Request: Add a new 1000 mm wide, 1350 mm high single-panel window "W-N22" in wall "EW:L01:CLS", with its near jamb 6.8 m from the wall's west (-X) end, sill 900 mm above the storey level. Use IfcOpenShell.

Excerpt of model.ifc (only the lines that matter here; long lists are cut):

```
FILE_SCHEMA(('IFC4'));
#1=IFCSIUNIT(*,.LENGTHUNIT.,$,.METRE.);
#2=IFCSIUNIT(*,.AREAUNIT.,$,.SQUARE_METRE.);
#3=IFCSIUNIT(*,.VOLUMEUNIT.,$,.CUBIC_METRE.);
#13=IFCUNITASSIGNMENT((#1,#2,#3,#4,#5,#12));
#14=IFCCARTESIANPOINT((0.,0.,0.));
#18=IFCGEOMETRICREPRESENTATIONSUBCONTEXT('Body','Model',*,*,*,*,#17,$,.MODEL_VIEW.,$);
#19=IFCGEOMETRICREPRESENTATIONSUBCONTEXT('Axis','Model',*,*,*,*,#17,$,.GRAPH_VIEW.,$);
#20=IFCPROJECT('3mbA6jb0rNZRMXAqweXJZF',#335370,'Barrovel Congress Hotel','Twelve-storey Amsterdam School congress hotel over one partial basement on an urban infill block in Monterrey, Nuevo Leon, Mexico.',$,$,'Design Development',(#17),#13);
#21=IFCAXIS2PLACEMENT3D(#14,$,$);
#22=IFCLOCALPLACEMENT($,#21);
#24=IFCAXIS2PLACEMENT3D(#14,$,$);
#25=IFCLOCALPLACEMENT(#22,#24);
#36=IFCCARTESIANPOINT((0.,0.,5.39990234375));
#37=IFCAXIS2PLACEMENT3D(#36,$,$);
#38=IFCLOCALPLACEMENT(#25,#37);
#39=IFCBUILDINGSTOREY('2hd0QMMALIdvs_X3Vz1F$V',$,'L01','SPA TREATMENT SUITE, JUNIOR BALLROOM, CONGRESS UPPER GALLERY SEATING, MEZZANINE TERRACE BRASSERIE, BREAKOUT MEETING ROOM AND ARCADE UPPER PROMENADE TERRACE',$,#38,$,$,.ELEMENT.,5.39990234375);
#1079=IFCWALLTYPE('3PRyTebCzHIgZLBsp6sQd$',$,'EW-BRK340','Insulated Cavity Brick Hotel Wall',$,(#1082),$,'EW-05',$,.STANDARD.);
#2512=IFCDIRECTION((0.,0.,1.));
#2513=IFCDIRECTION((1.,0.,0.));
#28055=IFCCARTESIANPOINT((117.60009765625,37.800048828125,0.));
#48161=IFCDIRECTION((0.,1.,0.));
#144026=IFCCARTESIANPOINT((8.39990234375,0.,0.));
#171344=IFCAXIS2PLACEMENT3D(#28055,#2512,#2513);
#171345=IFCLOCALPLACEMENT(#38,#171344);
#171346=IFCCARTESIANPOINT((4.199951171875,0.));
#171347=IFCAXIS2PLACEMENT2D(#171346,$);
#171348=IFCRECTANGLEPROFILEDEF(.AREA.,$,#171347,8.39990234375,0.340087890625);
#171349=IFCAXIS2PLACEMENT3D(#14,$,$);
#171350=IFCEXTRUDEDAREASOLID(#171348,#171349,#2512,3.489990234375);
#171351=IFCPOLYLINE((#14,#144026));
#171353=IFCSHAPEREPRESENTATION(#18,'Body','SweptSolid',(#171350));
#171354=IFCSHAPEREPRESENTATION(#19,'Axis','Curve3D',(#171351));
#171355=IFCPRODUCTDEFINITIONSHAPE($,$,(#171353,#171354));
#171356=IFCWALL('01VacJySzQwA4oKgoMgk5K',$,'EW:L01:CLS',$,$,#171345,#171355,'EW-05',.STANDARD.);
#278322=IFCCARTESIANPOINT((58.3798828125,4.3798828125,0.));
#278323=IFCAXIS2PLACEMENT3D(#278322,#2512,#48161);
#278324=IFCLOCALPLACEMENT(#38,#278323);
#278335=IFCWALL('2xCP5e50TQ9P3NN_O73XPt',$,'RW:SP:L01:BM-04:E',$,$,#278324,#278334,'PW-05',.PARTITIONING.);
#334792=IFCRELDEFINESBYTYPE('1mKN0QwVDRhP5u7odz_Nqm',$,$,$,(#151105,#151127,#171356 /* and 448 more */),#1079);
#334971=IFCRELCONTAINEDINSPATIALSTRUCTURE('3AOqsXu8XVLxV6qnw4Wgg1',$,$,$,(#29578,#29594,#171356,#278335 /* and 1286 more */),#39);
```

```python
import numpy as np
import ifcopenshell
import ifcopenshell.api.feature
import ifcopenshell.api.geometry
import ifcopenshell.api.root
import ifcopenshell.api.spatial
import ifcopenshell.geom
import ifcopenshell.util.element
import ifcopenshell.util.placement
import ifcopenshell.util.representation
import ifcopenshell.util.shape
import ifcopenshell.util.unit

model = ifcopenshell.open("model.ifc")
unit_scale = ifcopenshell.util.unit.calculate_unit_scale(model)
settings = ifcopenshell.geom.settings()


def volume(element):
    """Net volume in cubic metres, openings subtracted."""
    shape = ifcopenshell.geom.create_shape(settings, element)
    return ifcopenshell.util.shape.get_volume(shape.geometry)


wall = model.by_guid("01VacJySzQwA4oKgoMgk5K")
storey = ifcopenshell.util.element.get_container(wall, ifc_class="IfcBuildingStorey")
context = ifcopenshell.util.representation.get_context(model, "Model", "Body", "MODEL_VIEW")
before = volume(wall)

width, height, from_end, sill = 1, 1.35, 6.8, 0.9  # metres

# The wall runs along its own X axis, and the end named is its -X end.
wall_shape = ifcopenshell.geom.create_shape(settings, wall)
x, y, z = ifcopenshell.util.shape.get_vertices(wall_shape.geometry).T
start = x.min() + from_end
face, thickness = float(y.min()), float(y.max() - y.min())
wall_matrix = ifcopenshell.util.placement.get_local_placement(wall.ObjectPlacement)
level = ifcopenshell.util.placement.get_local_placement(storey.ObjectPlacement)[2, 3]


def in_wall(x, y):
    """Placement at x, y metres in the wall's axes, at sill height."""
    matrix = wall_matrix.copy()
    matrix[:, 3] = wall_matrix @ np.array([x / unit_scale, y / unit_scale, 0.0, 1.0])
    matrix[2, 3] = level + sill / unit_scale
    return matrix


# Opening: a box that overshoots both wall faces by 50 mm.
opening = ifcopenshell.api.root.create_entity(model, ifc_class="IfcOpeningElement", predefined_type="OPENING")
box = ifcopenshell.api.geometry.add_wall_representation(
    model, context=context, length=width, height=height, thickness=thickness + 0.1
)
ifcopenshell.api.geometry.assign_representation(model, product=opening, representation=box)
ifcopenshell.api.geometry.edit_object_placement(model, product=opening, matrix=in_wall(start, face - 0.05), is_si=False)
ifcopenshell.api.feature.add_feature(model, feature=opening, element=wall)

window = ifcopenshell.api.root.create_entity(model, ifc_class="IfcWindow", name="W-N22", predefined_type="WINDOW")
window.OverallWidth, window.OverallHeight = width / unit_scale, height / unit_scale
window.PartitioningType = "SINGLE_PANEL"
body = ifcopenshell.api.geometry.add_window_representation(
    model,
    context=context,
    overall_width=window.OverallWidth,
    overall_height=window.OverallHeight,
    partition_type="SINGLE_PANEL",
)
ifcopenshell.api.geometry.assign_representation(model, product=window, representation=body)
ifcopenshell.api.spatial.assign_container(model, products=[window], relating_structure=storey)
ifcopenshell.api.feature.add_filling(model, opening=opening, element=window)

# Centre the window in the wall's thickness.
ifcopenshell.api.geometry.edit_object_placement(model, product=window, matrix=in_wall(start, face), is_si=False)
window_shape = ifcopenshell.geom.create_shape(settings, window)
depth = ifcopenshell.util.shape.get_vertices(window_shape.geometry)[:, 1]
offset = face + thickness / 2 - (depth.min() + depth.max()) / 2
ifcopenshell.api.geometry.edit_object_placement(model, product=window, matrix=in_wall(start, offset), is_si=False)

after = volume(wall)

print(f"wall volume {before:.3f} -> {after:.3f} m3")

model.write("model_v2.ifc")
```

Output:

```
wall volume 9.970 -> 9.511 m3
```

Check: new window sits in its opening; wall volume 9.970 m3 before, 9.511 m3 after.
